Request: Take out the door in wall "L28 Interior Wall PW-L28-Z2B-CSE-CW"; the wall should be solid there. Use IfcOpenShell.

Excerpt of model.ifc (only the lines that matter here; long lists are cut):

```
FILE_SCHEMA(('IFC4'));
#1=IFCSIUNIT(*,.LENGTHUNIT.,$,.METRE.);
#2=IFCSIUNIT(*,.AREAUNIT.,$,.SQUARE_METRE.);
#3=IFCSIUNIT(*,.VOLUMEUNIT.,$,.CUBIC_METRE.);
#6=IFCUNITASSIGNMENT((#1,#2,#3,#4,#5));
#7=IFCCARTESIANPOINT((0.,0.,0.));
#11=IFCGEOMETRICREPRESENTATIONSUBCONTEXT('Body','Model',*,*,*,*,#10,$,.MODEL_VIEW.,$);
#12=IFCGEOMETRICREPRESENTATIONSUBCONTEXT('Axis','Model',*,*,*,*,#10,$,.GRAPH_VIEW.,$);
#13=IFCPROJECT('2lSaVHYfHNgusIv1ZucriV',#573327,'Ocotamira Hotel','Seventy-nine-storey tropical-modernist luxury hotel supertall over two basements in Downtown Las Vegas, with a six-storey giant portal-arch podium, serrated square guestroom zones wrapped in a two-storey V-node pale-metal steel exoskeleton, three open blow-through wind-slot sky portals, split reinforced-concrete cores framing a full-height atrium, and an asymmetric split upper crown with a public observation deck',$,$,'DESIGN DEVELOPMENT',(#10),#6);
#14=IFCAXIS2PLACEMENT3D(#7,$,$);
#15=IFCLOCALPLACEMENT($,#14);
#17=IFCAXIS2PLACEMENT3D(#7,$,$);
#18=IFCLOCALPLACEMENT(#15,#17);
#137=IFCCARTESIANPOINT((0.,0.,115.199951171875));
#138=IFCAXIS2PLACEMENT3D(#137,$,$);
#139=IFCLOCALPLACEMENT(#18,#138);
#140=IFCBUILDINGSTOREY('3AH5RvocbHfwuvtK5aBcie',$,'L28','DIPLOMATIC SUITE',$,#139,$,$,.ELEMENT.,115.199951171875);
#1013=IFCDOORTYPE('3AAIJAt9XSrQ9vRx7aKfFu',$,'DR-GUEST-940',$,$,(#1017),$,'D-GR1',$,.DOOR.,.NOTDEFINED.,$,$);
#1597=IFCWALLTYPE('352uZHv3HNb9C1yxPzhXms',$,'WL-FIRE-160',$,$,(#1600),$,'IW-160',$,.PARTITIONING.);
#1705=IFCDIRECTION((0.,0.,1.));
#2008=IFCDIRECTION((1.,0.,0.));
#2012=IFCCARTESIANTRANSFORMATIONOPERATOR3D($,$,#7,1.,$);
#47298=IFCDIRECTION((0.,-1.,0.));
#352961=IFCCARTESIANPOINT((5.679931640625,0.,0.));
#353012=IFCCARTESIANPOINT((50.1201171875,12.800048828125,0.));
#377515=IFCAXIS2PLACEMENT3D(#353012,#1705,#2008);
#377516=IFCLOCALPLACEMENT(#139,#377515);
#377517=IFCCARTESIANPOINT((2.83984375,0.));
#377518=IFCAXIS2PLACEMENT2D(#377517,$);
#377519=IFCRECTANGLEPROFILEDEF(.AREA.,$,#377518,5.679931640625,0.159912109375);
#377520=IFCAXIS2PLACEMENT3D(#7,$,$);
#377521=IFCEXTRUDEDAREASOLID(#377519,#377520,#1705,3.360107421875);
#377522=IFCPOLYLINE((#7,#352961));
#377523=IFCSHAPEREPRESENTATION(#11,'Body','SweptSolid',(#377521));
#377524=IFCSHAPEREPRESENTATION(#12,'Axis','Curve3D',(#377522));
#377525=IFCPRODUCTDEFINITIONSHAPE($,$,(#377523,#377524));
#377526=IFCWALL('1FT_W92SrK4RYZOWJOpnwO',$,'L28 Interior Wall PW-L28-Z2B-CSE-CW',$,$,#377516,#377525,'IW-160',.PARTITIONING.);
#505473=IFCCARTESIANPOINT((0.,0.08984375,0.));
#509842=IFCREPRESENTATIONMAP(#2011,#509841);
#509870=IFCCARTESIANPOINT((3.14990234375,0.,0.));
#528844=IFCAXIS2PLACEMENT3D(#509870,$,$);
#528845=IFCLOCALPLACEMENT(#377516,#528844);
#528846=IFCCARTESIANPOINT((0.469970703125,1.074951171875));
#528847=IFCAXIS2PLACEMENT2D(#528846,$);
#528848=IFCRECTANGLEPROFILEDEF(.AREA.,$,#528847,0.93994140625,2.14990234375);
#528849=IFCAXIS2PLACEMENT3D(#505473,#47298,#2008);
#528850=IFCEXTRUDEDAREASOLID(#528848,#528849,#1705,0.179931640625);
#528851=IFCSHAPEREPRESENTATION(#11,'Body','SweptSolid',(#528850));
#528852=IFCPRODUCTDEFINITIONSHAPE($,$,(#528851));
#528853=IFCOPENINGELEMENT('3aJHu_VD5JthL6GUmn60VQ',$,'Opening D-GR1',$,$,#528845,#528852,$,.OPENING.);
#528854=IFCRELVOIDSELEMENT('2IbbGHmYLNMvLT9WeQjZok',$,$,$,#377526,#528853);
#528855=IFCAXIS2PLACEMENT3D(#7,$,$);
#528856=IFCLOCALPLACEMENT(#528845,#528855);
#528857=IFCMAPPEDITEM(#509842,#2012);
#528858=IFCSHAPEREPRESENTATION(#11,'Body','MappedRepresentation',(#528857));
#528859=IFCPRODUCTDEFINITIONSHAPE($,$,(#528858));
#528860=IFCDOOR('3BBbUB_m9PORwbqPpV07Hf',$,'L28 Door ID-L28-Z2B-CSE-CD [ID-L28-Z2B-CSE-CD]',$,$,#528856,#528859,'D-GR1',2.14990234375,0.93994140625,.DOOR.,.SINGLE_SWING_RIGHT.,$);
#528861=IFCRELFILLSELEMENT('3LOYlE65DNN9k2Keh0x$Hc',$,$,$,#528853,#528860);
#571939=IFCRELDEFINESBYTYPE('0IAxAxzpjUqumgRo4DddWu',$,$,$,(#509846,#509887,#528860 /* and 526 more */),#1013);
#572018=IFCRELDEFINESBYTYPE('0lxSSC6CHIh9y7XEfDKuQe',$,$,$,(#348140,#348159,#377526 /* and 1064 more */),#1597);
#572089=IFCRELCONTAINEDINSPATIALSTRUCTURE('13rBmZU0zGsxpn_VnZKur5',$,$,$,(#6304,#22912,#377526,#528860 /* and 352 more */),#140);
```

```python
import ifcopenshell
import ifcopenshell.api.feature
import ifcopenshell.api.root
import ifcopenshell.geom
import ifcopenshell.util.shape

model = ifcopenshell.open("model.ifc")
settings = ifcopenshell.geom.settings()


def volume(element):
    """Net volume in cubic metres, openings subtracted."""
    shape = ifcopenshell.geom.create_shape(settings, element)
    return ifcopenshell.util.shape.get_volume(shape.geometry)


door = model.by_id(528860)
opening = door.FillsVoids[0].RelatingOpeningElement
wall = opening.VoidsElements[0].RelatingBuildingElement
before = volume(wall)

ifcopenshell.api.root.remove_product(model, product=door)
ifcopenshell.api.feature.remove_feature(model, feature=opening)

after = volume(wall)

print(f"wall volume {before:.3f} -> {after:.3f} m3")

model.write("model-out.ifc")
```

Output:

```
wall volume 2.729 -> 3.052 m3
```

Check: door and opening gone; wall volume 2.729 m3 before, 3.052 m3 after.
